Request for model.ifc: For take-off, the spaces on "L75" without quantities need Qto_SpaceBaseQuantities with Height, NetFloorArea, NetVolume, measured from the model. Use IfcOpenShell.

First a look at what the model holds.

```python
import ifcopenshell
import ifcopenshell.util.element
import ifcopenshell.util.unit

model = ifcopenshell.open("model.ifc")
print(model.schema)
for unit_type in ("LENGTHUNIT", "AREAUNIT", "VOLUMEUNIT"):
    print(unit_type, ifcopenshell.util.unit.calculate_unit_scale(model, unit_type))
storey = next(s for s in model.by_type("IfcBuildingStorey") if s.Name == "L75")
spaces = [e for e in ifcopenshell.util.element.get_decomposition(storey) if e.is_a("IfcSpace")]
for e in sorted(spaces, key=lambda e: e.id()):
    print(e.id(), e.is_a(), e.Name, list(ifcopenshell.util.element.get_psets(e, qtos_only=True)), sep=" | ")
```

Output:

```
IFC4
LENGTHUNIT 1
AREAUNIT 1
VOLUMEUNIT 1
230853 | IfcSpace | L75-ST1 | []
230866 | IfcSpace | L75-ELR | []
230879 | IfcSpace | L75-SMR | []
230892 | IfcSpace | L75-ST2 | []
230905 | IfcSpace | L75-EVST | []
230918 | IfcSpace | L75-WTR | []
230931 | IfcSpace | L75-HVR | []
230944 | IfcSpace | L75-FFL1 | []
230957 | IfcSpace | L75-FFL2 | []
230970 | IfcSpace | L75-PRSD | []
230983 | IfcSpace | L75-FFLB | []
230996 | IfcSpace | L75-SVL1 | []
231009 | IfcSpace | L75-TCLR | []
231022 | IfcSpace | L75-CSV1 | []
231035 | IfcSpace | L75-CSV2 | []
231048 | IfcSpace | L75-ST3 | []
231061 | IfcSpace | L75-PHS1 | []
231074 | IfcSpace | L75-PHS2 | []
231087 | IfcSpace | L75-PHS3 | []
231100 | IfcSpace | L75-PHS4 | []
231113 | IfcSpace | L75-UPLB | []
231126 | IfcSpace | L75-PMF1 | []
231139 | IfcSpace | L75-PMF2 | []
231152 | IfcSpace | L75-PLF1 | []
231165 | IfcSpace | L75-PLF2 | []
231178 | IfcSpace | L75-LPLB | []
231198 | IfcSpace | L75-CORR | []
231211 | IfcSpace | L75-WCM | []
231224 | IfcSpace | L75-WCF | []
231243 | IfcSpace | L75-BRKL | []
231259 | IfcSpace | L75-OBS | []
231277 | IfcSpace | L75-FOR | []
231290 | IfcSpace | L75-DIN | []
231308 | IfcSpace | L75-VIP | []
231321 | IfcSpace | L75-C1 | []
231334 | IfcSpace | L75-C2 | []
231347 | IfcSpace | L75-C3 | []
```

```python
import ifcopenshell
import ifcopenshell.api.pset
import ifcopenshell.geom
import ifcopenshell.util.element
import ifcopenshell.util.shape
import ifcopenshell.util.unit

model = ifcopenshell.open("model.ifc")
unit_scale = ifcopenshell.util.unit.calculate_unit_scale(model)
area_scale = ifcopenshell.util.unit.calculate_unit_scale(model, "AREAUNIT")
volume_scale = ifcopenshell.util.unit.calculate_unit_scale(model, "VOLUMEUNIT")
settings = ifcopenshell.geom.settings()

storey = next(s for s in model.by_type("IfcBuildingStorey") if s.Name == "L75")
spaces = [e for e in ifcopenshell.util.element.get_decomposition(storey) if e.is_a("IfcSpace")]

for e in sorted(spaces, key=lambda e: e.id()):
    if ifcopenshell.util.element.get_psets(e, qtos_only=True, should_inherit=False):
        continue
    # Geometry comes back in metres, in the element's own axes.
    shape = ifcopenshell.geom.create_shape(settings, e)
    values = {
        "Height": ifcopenshell.util.shape.get_z(shape.geometry) / unit_scale,
        "NetFloorArea": ifcopenshell.util.shape.get_footprint_area(shape.geometry) / area_scale,
        "NetVolume": ifcopenshell.util.shape.get_volume(shape.geometry) / volume_scale,
    }
    qto = ifcopenshell.api.pset.add_qto(model, product=e, name="Qto_SpaceBaseQuantities")
    ifcopenshell.api.pset.edit_qto(model, qto=qto, properties=values)
    print(e.id(), {k: round(v, 3) for k, v in values.items()})

model.write("model_v2.ifc")
```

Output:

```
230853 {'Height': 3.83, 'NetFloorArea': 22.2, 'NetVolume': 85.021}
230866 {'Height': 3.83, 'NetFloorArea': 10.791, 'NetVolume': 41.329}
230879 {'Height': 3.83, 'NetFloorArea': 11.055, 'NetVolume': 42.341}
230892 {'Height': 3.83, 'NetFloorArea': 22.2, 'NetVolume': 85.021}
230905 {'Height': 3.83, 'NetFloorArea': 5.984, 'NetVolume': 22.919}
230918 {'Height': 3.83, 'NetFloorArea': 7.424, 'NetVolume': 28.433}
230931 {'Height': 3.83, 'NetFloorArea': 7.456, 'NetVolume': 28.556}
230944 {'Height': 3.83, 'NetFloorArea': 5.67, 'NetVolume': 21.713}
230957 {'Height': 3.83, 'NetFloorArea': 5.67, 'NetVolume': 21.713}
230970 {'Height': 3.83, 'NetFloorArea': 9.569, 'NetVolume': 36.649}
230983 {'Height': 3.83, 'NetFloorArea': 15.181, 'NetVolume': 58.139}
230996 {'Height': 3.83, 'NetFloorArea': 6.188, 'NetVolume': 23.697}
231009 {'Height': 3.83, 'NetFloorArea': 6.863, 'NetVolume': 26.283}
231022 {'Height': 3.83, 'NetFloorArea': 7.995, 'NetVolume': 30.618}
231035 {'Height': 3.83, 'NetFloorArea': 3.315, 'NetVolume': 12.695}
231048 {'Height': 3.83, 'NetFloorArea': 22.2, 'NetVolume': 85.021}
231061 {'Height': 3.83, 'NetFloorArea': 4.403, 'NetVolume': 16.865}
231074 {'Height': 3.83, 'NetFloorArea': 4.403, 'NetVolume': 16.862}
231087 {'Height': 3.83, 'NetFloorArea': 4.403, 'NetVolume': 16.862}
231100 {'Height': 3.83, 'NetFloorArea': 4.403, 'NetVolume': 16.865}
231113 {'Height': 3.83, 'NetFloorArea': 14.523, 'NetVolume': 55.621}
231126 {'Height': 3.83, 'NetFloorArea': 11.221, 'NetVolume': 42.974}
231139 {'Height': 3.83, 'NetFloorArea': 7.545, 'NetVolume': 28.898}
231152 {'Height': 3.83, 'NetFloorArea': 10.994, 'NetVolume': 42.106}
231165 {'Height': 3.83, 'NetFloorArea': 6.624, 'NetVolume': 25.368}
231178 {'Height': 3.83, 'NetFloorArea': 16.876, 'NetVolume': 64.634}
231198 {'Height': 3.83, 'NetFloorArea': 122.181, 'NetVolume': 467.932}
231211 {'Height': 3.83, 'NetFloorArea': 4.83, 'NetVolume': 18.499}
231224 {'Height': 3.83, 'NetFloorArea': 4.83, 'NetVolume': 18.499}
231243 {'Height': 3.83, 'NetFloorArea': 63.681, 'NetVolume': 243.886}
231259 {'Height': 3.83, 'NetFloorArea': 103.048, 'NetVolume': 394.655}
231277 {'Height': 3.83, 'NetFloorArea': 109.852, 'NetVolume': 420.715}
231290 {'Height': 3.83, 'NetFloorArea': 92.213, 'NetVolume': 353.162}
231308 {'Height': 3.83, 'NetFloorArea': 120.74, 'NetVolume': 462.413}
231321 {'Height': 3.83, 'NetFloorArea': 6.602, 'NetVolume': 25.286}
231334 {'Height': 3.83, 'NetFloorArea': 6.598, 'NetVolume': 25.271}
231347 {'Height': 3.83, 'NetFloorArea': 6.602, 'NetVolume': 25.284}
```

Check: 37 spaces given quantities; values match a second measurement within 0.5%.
